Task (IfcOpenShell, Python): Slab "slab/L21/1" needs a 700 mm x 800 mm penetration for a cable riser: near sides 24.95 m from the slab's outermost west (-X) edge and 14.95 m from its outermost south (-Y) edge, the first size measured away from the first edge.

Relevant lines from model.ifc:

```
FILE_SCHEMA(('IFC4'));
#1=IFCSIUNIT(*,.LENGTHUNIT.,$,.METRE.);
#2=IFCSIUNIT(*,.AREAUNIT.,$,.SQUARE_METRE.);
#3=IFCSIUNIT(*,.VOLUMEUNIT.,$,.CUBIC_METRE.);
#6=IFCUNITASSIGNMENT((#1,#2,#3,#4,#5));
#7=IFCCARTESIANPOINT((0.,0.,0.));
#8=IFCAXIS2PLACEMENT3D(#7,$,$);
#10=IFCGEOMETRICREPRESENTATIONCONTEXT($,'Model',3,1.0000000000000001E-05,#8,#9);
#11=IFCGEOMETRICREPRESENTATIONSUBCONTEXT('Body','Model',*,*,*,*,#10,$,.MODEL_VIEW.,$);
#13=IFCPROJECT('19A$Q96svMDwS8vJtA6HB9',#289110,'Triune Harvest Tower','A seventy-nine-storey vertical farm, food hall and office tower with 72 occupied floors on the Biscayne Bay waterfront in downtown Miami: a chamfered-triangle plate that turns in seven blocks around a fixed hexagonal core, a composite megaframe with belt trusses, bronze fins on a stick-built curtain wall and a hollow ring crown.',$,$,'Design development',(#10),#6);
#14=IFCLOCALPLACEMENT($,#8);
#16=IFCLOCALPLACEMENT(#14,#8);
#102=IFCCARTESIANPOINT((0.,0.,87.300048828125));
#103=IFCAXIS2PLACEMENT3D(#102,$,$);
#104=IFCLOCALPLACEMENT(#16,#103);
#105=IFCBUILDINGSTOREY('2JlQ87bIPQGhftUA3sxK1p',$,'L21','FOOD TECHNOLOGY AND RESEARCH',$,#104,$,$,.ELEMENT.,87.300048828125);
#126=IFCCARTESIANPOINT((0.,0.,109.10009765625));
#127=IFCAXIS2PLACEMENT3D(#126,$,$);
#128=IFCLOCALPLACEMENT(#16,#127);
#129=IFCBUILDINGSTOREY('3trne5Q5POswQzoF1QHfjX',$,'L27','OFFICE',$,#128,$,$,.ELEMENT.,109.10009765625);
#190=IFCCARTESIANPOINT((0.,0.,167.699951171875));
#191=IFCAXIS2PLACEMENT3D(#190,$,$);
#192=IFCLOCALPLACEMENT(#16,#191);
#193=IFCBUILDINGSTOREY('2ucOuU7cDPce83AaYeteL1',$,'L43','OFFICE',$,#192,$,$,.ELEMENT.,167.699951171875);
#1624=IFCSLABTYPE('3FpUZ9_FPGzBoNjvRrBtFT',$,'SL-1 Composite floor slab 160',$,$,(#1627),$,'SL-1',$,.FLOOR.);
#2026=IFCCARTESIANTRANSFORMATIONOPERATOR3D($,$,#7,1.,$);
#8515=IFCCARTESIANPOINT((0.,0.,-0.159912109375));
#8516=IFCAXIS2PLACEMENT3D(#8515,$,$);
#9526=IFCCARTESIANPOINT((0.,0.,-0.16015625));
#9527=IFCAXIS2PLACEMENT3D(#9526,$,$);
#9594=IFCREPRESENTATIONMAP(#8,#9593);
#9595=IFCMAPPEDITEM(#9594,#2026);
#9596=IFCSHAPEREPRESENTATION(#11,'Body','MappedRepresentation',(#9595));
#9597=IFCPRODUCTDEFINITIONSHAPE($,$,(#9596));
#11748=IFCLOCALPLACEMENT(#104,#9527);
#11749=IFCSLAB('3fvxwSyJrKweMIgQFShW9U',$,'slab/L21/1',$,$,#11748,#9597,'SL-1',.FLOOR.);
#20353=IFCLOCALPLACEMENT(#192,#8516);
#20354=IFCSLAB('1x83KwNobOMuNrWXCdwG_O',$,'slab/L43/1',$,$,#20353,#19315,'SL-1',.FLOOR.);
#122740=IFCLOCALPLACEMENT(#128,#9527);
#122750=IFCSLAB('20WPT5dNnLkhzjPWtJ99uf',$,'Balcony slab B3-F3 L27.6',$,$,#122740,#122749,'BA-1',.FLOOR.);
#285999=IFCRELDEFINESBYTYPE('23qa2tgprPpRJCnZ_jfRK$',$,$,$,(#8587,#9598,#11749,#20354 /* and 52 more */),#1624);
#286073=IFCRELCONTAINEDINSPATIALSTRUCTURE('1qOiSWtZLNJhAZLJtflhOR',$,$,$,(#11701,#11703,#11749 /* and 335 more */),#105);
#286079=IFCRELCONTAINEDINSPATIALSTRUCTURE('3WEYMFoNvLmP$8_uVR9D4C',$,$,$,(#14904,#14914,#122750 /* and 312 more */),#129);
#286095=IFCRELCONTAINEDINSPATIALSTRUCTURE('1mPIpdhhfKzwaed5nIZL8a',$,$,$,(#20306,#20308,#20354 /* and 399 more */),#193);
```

```python
import numpy as np
import ifcopenshell
import ifcopenshell.api.feature
import ifcopenshell.api.geometry
import ifcopenshell.api.root
import ifcopenshell.geom
import ifcopenshell.util.placement
import ifcopenshell.util.representation
import ifcopenshell.util.shape
import ifcopenshell.util.unit

model = ifcopenshell.open("model.ifc")
unit_scale = ifcopenshell.util.unit.calculate_unit_scale(model)
settings = ifcopenshell.geom.settings()


def volume(element):
    """Net volume in cubic metres, openings subtracted."""
    shape = ifcopenshell.geom.create_shape(settings, element)
    return ifcopenshell.util.shape.get_volume(shape.geometry)


slab = model.by_guid("3fvxwSyJrKweMIgQFShW9U")
before = volume(slab)

# Extent in the slab's own axes, in metres. The edges named are its -X and -Y sides.
slab_shape = ifcopenshell.geom.create_shape(settings, slab)
vertices = ifcopenshell.util.shape.get_vertices(slab_shape.geometry)
x_min, y_min, bottom = vertices.min(axis=0)
top = vertices[:, 2].max()

opening = ifcopenshell.api.root.create_entity(model, ifc_class="IfcOpeningElement", name="Cable riser opening", predefined_type="OPENING")
context = ifcopenshell.util.representation.get_context(model, "Model", "Body", "MODEL_VIEW")
width, depth = 0.7, 0.8
outline = [(0.0, 0.0), (width, 0.0), (width, depth), (0.0, depth), (0.0, 0.0)]
# Overshoot both faces by 50 mm so the cut is clean.
shape = ifcopenshell.api.geometry.add_slab_representation(
    model, context=context, depth=top - bottom + 0.1, polyline=outline
)
ifcopenshell.api.geometry.assign_representation(model, product=opening, representation=shape)

matrix = ifcopenshell.util.placement.get_local_placement(slab.ObjectPlacement)
matrix[:, 3] = matrix @ np.append(np.array([x_min + 24.95, y_min + 14.95, bottom - 0.05]) / unit_scale, 1.0)
ifcopenshell.api.geometry.edit_object_placement(model, product=opening, matrix=matrix, is_si=False)
ifcopenshell.api.feature.add_feature(model, feature=opening, element=slab)

after = volume(slab)

print(f"slab volume {before:.3f} -> {after:.3f} m3")

model.write("model-out.ifc")
```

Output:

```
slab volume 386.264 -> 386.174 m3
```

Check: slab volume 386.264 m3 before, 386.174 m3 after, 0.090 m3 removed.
